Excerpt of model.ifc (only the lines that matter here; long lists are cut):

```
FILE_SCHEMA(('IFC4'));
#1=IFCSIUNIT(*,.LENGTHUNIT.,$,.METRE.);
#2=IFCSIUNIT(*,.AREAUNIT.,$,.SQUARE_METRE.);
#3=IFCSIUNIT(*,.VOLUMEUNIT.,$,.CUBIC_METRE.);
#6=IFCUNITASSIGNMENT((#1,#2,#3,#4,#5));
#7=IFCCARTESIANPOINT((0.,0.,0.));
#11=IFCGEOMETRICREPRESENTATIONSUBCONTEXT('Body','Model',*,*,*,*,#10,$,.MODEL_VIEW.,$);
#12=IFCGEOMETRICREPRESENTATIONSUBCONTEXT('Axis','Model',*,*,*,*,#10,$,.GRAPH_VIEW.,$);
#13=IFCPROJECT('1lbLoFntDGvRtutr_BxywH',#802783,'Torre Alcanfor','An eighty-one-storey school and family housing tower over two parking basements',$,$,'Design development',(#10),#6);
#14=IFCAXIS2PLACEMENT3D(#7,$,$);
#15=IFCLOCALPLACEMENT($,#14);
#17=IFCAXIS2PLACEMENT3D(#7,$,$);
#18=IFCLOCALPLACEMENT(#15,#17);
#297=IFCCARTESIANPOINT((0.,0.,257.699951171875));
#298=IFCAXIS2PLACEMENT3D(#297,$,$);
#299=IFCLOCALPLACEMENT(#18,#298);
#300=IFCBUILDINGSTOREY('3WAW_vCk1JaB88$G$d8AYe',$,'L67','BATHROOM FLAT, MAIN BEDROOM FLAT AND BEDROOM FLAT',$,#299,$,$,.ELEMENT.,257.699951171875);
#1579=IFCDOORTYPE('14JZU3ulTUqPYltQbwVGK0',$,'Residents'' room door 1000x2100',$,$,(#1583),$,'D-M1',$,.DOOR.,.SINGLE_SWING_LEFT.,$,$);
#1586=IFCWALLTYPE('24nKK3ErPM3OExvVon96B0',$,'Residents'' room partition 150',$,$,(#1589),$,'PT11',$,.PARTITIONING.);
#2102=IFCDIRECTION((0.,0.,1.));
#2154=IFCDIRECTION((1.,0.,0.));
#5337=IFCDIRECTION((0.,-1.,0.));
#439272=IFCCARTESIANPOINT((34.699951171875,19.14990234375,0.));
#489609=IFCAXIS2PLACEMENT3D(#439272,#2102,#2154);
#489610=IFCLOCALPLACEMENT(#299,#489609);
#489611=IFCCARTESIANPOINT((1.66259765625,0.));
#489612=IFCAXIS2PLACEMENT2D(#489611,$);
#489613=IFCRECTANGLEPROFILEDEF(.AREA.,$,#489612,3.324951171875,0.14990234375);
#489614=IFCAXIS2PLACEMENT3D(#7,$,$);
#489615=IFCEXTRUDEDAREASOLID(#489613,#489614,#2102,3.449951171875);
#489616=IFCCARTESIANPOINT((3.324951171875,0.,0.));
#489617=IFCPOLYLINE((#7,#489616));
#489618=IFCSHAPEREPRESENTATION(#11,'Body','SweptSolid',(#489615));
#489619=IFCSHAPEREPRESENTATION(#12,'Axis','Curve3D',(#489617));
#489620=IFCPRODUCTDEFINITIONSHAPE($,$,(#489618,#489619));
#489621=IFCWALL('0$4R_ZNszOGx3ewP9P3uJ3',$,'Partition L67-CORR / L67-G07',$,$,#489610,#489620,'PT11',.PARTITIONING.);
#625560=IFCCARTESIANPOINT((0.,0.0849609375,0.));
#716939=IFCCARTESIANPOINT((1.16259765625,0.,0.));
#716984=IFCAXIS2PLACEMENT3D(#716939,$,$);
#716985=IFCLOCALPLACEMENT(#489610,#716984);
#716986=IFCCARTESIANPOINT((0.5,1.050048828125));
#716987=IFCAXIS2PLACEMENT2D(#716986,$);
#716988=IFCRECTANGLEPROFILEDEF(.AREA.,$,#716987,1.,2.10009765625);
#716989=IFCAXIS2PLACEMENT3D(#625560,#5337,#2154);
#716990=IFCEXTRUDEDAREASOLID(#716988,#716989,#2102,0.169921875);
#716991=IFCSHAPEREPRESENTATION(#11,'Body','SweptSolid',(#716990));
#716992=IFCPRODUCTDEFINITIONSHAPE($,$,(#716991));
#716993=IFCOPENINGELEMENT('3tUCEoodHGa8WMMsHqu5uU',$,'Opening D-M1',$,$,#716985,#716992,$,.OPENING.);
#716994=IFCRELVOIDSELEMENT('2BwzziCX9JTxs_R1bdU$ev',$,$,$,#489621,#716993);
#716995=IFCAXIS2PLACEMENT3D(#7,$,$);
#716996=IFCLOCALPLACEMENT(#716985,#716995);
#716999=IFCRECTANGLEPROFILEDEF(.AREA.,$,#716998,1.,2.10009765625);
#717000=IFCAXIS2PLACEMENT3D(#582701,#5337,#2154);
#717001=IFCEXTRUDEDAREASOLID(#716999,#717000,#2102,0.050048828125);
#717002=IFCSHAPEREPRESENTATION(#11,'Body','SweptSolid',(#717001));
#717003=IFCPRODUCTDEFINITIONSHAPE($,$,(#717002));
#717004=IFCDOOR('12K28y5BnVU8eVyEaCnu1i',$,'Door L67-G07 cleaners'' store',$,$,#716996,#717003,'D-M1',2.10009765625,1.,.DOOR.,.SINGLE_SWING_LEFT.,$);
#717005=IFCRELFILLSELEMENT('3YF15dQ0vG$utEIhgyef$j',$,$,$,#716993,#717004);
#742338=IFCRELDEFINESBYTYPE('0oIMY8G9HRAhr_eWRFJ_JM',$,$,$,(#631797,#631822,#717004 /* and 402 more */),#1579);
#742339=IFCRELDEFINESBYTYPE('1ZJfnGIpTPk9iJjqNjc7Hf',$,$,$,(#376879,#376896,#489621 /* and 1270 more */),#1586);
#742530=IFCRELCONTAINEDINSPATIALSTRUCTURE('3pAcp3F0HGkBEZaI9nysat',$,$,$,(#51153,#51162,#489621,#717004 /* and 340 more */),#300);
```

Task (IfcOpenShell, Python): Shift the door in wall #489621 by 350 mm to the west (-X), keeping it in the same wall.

```python
import ifcopenshell
import ifcopenshell.api.geometry
import ifcopenshell.util.placement
import ifcopenshell.util.unit

model = ifcopenshell.open("model.ifc")
unit_scale = ifcopenshell.util.unit.calculate_unit_scale(model)

door = model.by_guid("12K28y5BnVU8eVyEaCnu1i")
opening = door.FillsVoids[0].RelatingOpeningElement
wall = opening.VoidsElements[0].RelatingBuildingElement

wall_matrix = ifcopenshell.util.placement.get_local_placement(wall.ObjectPlacement)
shift = wall_matrix[:3, 0] * -0.35 / unit_scale
before = ifcopenshell.util.placement.get_local_placement(door.ObjectPlacement)[:3, 3].copy()

# The door is placed relative to its opening, so it follows when the opening moves.
matrix = ifcopenshell.util.placement.get_local_placement(opening.ObjectPlacement)
matrix[:3, 3] += shift
ifcopenshell.api.geometry.edit_object_placement(
    model, product=opening, matrix=matrix, is_si=False, should_transform_children=True
)

after = ifcopenshell.util.placement.get_local_placement(door.ObjectPlacement)[:3, 3]
print("door moved by", (after - before).round(3) + 0.0)

model.write("model_rev.ifc")
```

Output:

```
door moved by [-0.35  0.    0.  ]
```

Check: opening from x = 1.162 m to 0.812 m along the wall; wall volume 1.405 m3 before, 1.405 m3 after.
